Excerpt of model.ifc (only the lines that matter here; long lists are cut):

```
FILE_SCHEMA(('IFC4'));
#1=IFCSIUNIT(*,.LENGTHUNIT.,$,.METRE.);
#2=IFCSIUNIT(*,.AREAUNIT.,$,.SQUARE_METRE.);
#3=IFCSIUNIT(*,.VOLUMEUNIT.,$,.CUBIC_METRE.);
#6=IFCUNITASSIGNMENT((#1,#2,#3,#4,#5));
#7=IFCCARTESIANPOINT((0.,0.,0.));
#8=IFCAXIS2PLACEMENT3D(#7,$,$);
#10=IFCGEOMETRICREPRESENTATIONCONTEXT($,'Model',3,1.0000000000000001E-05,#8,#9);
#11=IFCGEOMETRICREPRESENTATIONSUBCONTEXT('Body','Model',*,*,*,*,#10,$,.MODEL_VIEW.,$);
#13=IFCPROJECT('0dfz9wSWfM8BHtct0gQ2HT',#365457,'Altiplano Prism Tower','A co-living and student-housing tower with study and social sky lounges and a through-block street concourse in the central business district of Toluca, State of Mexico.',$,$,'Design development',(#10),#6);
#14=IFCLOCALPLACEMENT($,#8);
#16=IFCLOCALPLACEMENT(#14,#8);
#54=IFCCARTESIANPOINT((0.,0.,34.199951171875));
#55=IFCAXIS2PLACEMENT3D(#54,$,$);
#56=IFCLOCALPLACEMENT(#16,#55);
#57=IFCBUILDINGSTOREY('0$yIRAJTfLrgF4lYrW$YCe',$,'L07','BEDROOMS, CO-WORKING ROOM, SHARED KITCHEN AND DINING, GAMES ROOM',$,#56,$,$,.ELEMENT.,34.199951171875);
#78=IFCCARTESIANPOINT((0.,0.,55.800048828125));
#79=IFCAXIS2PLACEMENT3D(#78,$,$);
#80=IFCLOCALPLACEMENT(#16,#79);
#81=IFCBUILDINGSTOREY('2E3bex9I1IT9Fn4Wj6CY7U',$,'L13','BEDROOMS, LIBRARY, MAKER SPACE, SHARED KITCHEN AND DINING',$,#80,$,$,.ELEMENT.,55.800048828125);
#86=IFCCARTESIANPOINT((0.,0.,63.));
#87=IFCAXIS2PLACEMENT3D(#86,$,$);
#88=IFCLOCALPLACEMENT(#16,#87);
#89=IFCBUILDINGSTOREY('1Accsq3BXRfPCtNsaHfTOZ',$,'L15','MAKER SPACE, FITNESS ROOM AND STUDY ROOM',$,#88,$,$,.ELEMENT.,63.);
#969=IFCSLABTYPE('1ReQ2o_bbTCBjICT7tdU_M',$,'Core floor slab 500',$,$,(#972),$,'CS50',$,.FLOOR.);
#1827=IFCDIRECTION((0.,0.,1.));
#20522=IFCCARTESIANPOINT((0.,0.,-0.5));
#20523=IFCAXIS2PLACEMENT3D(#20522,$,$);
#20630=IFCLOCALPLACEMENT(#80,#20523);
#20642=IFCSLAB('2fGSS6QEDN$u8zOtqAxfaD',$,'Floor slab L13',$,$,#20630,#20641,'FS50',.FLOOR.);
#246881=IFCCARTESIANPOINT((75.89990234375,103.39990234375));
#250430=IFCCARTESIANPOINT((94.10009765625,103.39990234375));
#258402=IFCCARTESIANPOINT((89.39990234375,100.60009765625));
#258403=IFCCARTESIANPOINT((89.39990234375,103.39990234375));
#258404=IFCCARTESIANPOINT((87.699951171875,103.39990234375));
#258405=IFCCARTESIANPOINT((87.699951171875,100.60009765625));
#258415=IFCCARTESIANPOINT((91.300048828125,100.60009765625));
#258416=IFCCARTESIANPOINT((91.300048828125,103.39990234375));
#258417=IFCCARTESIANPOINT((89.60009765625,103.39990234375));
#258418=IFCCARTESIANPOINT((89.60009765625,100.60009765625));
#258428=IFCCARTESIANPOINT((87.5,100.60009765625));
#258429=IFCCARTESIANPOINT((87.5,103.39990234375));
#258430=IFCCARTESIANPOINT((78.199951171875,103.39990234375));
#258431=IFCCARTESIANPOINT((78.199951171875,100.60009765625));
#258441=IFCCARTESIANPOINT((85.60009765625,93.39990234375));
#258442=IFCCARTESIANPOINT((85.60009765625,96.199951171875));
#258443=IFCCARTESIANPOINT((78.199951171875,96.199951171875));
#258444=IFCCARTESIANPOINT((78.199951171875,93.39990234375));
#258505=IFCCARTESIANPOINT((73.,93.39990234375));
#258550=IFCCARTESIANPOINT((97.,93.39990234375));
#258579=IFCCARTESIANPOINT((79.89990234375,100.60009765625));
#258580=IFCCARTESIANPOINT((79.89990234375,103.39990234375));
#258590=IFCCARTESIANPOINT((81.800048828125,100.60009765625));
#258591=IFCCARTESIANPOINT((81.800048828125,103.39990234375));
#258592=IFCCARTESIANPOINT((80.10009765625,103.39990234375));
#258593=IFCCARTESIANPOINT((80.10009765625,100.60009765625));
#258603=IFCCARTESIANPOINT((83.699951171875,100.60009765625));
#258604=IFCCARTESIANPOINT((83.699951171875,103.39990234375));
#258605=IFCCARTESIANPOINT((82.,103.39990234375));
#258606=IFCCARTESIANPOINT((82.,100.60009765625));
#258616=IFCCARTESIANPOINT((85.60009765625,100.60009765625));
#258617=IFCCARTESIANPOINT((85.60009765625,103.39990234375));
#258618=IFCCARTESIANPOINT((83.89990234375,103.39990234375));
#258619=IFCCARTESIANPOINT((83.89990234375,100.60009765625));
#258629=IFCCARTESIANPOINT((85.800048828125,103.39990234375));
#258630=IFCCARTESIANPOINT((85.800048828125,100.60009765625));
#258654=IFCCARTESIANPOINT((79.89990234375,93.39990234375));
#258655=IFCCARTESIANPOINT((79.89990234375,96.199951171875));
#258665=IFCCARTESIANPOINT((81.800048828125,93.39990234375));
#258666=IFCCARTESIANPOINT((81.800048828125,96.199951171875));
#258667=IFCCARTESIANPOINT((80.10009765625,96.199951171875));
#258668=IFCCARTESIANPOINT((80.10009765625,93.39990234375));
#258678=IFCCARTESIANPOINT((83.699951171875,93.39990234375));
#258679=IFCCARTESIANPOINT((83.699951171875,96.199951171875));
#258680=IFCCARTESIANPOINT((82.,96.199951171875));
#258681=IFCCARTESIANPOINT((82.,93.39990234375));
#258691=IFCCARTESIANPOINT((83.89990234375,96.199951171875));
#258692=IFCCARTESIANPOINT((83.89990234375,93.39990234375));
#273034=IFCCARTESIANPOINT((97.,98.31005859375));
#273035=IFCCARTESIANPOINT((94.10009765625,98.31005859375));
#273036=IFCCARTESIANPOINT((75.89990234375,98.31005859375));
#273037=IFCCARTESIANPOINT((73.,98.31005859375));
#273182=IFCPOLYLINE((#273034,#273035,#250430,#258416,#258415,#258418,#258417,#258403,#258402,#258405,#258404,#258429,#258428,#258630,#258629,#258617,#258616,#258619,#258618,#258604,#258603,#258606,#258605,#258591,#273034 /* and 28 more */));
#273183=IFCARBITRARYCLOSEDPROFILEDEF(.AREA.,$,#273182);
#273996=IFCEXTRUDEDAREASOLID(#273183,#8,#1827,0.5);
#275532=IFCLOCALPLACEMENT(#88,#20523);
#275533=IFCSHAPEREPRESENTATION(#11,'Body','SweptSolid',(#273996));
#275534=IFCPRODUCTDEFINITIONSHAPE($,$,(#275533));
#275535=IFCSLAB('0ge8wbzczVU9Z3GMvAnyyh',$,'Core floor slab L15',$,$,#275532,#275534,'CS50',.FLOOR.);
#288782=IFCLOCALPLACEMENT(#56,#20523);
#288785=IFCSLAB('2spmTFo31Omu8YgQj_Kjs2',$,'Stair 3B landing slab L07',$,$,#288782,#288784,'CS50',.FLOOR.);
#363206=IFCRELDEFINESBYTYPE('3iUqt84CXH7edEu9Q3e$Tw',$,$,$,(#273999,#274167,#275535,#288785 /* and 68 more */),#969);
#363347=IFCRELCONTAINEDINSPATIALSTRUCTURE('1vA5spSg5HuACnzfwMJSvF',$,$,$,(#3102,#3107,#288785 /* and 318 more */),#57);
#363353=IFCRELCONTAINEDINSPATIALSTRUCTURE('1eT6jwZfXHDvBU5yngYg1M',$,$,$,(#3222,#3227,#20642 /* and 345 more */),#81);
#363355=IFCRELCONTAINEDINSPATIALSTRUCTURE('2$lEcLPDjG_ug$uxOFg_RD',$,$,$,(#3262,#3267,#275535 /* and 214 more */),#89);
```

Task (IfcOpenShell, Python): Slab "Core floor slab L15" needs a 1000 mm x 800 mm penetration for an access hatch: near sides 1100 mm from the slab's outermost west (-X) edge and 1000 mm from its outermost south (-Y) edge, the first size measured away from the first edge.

```python
import numpy as np
import ifcopenshell
import ifcopenshell.api.feature
import ifcopenshell.api.geometry
import ifcopenshell.api.root
import ifcopenshell.geom
import ifcopenshell.util.placement
import ifcopenshell.util.representation
import ifcopenshell.util.shape
import ifcopenshell.util.unit

model = ifcopenshell.open("model.ifc")
unit_scale = ifcopenshell.util.unit.calculate_unit_scale(model)
settings = ifcopenshell.geom.settings()


def volume(element):
    """Net volume in cubic metres, openings subtracted."""
    shape = ifcopenshell.geom.create_shape(settings, element)
    return ifcopenshell.util.shape.get_volume(shape.geometry)


slab = model.by_guid("0ge8wbzczVU9Z3GMvAnyyh")
before = volume(slab)

# Extent in the slab's own axes, in metres. The edges named are its -X and -Y sides.
slab_shape = ifcopenshell.geom.create_shape(settings, slab)
vertices = ifcopenshell.util.shape.get_vertices(slab_shape.geometry)
x_min, y_min, bottom = vertices.min(axis=0)
top = vertices[:, 2].max()

opening = ifcopenshell.api.root.create_entity(model, ifc_class="IfcOpeningElement", name="Access hatch opening", predefined_type="OPENING")
context = ifcopenshell.util.representation.get_context(model, "Model", "Body", "MODEL_VIEW")
width, depth = 1, 0.8
outline = [(0.0, 0.0), (width, 0.0), (width, depth), (0.0, depth), (0.0, 0.0)]
# Overshoot both faces by 50 mm so the cut is clean.
shape = ifcopenshell.api.geometry.add_slab_representation(
    model, context=context, depth=top - bottom + 0.1, polyline=outline
)
ifcopenshell.api.geometry.assign_representation(model, product=opening, representation=shape)

matrix = ifcopenshell.util.placement.get_local_placement(slab.ObjectPlacement)
matrix[:, 3] = matrix @ np.append(np.array([x_min + 1.1, y_min + 1, bottom - 0.05]) / unit_scale, 1.0)
ifcopenshell.api.geometry.edit_object_placement(model, product=opening, matrix=matrix, is_si=False)
ifcopenshell.api.feature.add_feature(model, feature=opening, element=slab)

after = volume(slab)

print(f"slab volume {before:.3f} -> {after:.3f} m3")

model.write("model-out.ifc")
```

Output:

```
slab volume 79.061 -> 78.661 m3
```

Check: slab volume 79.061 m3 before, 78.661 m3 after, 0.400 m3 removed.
